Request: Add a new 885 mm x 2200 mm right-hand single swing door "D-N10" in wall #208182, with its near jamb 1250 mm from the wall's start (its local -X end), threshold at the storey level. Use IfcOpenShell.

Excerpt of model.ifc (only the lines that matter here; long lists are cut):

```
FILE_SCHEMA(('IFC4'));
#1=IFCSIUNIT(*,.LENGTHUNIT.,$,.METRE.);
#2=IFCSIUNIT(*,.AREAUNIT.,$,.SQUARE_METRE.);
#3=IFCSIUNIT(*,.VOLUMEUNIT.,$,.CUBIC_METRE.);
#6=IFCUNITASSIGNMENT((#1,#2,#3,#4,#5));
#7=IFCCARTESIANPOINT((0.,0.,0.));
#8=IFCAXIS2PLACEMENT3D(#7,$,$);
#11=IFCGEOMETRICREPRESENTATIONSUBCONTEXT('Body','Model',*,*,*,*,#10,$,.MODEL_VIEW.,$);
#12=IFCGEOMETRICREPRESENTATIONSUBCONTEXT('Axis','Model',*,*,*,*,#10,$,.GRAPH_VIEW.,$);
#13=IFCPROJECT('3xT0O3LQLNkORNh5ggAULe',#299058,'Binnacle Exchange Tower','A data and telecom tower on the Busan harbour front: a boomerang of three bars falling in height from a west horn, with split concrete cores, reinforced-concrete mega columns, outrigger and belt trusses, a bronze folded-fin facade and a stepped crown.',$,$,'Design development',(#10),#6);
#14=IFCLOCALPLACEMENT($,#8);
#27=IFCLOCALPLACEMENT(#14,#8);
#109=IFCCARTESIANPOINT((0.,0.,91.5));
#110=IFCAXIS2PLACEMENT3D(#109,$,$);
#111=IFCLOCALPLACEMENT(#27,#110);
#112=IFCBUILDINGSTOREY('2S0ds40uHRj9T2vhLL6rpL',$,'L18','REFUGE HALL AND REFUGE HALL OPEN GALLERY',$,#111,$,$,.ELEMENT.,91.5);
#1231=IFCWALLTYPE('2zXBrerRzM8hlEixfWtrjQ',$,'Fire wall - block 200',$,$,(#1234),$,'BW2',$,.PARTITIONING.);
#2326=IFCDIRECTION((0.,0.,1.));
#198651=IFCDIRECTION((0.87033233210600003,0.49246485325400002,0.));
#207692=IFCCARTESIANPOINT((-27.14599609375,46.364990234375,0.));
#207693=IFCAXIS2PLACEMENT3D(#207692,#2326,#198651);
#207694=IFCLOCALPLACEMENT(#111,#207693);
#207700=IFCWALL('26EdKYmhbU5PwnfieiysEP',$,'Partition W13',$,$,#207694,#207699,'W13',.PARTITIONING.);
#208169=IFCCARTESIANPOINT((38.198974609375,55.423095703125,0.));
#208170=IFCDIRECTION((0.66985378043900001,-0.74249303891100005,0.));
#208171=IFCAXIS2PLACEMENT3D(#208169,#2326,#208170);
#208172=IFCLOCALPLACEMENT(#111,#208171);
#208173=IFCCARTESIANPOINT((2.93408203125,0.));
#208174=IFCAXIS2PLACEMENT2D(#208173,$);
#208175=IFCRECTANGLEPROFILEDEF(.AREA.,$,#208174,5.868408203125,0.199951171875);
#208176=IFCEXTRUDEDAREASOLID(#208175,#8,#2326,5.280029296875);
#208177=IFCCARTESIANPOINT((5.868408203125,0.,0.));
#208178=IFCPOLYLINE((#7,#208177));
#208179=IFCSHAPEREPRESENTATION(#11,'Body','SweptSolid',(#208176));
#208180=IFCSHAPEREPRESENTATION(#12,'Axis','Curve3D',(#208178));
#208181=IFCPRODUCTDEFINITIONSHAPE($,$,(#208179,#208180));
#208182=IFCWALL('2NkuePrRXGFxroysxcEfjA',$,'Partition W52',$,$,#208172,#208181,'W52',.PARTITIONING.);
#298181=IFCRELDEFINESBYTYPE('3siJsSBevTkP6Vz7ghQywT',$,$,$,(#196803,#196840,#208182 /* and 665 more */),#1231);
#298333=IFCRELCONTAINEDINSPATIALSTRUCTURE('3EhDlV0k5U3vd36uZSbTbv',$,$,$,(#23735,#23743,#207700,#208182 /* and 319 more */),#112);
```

```python
import numpy as np
import ifcopenshell
import ifcopenshell.api.feature
import ifcopenshell.api.geometry
import ifcopenshell.api.root
import ifcopenshell.api.spatial
import ifcopenshell.geom
import ifcopenshell.util.element
import ifcopenshell.util.placement
import ifcopenshell.util.representation
import ifcopenshell.util.shape
import ifcopenshell.util.unit

model = ifcopenshell.open("model.ifc")
unit_scale = ifcopenshell.util.unit.calculate_unit_scale(model)
settings = ifcopenshell.geom.settings()


def volume(element):
    """Net volume in cubic metres, openings subtracted."""
    shape = ifcopenshell.geom.create_shape(settings, element)
    return ifcopenshell.util.shape.get_volume(shape.geometry)


wall = model.by_guid("2NkuePrRXGFxroysxcEfjA")
storey = ifcopenshell.util.element.get_container(wall, ifc_class="IfcBuildingStorey")
context = ifcopenshell.util.representation.get_context(model, "Model", "Body", "MODEL_VIEW")
before = volume(wall)

width, height, from_end, sill = 0.885, 2.2, 1.25, 0.0  # metres

# The wall runs along its own X axis, and the end named is its -X end.
wall_shape = ifcopenshell.geom.create_shape(settings, wall)
x, y, z = ifcopenshell.util.shape.get_vertices(wall_shape.geometry).T
start = x.min() + from_end
face, thickness = float(y.min()), float(y.max() - y.min())
wall_matrix = ifcopenshell.util.placement.get_local_placement(wall.ObjectPlacement)
level = ifcopenshell.util.placement.get_local_placement(storey.ObjectPlacement)[2, 3]


def in_wall(x, y):
    """Placement at x, y metres in the wall's axes, at sill height."""
    matrix = wall_matrix.copy()
    matrix[:, 3] = wall_matrix @ np.array([x / unit_scale, y / unit_scale, 0.0, 1.0])
    matrix[2, 3] = level + sill / unit_scale
    return matrix


# Opening: a box that overshoots both wall faces by 50 mm.
opening = ifcopenshell.api.root.create_entity(model, ifc_class="IfcOpeningElement", predefined_type="OPENING")
box = ifcopenshell.api.geometry.add_wall_representation(
    model, context=context, length=width, height=height, thickness=thickness + 0.1
)
ifcopenshell.api.geometry.assign_representation(model, product=opening, representation=box)
ifcopenshell.api.geometry.edit_object_placement(model, product=opening, matrix=in_wall(start, face - 0.05), is_si=False)
ifcopenshell.api.feature.add_feature(model, feature=opening, element=wall)

door = ifcopenshell.api.root.create_entity(model, ifc_class="IfcDoor", name="D-N10", predefined_type="DOOR")
door.OverallWidth, door.OverallHeight = width / unit_scale, height / unit_scale
door.OperationType = "SINGLE_SWING_RIGHT"
body = ifcopenshell.api.geometry.add_door_representation(
    model,
    context=context,
    overall_width=door.OverallWidth,
    overall_height=door.OverallHeight,
    operation_type="SINGLE_SWING_RIGHT",
    lining_properties={"LiningDepth": thickness / unit_scale, "ThresholdDepth": thickness / unit_scale},
)
ifcopenshell.api.geometry.assign_representation(model, product=door, representation=body)
ifcopenshell.api.spatial.assign_container(model, products=[door], relating_structure=storey)
ifcopenshell.api.feature.add_filling(model, opening=opening, element=door)

# The lining spans the wall, so the door starts at the wall face.
ifcopenshell.api.geometry.edit_object_placement(model, product=door, matrix=in_wall(start, face), is_si=False)

after = volume(wall)

print(f"wall volume {before:.3f} -> {after:.3f} m3")

model.write("model_edited.ifc")
```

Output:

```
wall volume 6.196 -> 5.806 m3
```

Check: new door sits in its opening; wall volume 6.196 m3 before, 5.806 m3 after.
